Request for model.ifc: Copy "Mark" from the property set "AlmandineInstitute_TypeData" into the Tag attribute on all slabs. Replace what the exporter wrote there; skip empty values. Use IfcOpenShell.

First a look at what the model holds.

```python
import ifcopenshell
import ifcopenshell.util.element

model = ifcopenshell.open("model.ifc")
print(model.schema)
slabs = model.by_type("IfcSlab")
print(len(slabs), "slabs")
for e in slabs[:8]:
    source = ifcopenshell.util.element.get_pset(e, "AlmandineInstitute_TypeData", "Mark")
    target = e.Tag
    print(e.id(), repr(source), repr(target), sep=" | ")
```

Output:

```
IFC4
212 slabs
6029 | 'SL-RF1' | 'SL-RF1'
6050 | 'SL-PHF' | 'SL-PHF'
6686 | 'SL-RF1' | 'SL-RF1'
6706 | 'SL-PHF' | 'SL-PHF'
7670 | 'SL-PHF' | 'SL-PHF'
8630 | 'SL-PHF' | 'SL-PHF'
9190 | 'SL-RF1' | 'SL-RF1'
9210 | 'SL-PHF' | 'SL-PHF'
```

```python
import ifcopenshell
import ifcopenshell.util.element

model = ifcopenshell.open("model.ifc")

count = 0
for e in model.by_type("IfcSlab"):
    value = ifcopenshell.util.element.get_pset(e, "AlmandineInstitute_TypeData", "Mark")
    current = e.Tag
    if not value or not value.strip() or current == value:
        continue
    e.Tag = value
    count += 1

print(count, "slabs updated")

model.write("model-out.ifc")
```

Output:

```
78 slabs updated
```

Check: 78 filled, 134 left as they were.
